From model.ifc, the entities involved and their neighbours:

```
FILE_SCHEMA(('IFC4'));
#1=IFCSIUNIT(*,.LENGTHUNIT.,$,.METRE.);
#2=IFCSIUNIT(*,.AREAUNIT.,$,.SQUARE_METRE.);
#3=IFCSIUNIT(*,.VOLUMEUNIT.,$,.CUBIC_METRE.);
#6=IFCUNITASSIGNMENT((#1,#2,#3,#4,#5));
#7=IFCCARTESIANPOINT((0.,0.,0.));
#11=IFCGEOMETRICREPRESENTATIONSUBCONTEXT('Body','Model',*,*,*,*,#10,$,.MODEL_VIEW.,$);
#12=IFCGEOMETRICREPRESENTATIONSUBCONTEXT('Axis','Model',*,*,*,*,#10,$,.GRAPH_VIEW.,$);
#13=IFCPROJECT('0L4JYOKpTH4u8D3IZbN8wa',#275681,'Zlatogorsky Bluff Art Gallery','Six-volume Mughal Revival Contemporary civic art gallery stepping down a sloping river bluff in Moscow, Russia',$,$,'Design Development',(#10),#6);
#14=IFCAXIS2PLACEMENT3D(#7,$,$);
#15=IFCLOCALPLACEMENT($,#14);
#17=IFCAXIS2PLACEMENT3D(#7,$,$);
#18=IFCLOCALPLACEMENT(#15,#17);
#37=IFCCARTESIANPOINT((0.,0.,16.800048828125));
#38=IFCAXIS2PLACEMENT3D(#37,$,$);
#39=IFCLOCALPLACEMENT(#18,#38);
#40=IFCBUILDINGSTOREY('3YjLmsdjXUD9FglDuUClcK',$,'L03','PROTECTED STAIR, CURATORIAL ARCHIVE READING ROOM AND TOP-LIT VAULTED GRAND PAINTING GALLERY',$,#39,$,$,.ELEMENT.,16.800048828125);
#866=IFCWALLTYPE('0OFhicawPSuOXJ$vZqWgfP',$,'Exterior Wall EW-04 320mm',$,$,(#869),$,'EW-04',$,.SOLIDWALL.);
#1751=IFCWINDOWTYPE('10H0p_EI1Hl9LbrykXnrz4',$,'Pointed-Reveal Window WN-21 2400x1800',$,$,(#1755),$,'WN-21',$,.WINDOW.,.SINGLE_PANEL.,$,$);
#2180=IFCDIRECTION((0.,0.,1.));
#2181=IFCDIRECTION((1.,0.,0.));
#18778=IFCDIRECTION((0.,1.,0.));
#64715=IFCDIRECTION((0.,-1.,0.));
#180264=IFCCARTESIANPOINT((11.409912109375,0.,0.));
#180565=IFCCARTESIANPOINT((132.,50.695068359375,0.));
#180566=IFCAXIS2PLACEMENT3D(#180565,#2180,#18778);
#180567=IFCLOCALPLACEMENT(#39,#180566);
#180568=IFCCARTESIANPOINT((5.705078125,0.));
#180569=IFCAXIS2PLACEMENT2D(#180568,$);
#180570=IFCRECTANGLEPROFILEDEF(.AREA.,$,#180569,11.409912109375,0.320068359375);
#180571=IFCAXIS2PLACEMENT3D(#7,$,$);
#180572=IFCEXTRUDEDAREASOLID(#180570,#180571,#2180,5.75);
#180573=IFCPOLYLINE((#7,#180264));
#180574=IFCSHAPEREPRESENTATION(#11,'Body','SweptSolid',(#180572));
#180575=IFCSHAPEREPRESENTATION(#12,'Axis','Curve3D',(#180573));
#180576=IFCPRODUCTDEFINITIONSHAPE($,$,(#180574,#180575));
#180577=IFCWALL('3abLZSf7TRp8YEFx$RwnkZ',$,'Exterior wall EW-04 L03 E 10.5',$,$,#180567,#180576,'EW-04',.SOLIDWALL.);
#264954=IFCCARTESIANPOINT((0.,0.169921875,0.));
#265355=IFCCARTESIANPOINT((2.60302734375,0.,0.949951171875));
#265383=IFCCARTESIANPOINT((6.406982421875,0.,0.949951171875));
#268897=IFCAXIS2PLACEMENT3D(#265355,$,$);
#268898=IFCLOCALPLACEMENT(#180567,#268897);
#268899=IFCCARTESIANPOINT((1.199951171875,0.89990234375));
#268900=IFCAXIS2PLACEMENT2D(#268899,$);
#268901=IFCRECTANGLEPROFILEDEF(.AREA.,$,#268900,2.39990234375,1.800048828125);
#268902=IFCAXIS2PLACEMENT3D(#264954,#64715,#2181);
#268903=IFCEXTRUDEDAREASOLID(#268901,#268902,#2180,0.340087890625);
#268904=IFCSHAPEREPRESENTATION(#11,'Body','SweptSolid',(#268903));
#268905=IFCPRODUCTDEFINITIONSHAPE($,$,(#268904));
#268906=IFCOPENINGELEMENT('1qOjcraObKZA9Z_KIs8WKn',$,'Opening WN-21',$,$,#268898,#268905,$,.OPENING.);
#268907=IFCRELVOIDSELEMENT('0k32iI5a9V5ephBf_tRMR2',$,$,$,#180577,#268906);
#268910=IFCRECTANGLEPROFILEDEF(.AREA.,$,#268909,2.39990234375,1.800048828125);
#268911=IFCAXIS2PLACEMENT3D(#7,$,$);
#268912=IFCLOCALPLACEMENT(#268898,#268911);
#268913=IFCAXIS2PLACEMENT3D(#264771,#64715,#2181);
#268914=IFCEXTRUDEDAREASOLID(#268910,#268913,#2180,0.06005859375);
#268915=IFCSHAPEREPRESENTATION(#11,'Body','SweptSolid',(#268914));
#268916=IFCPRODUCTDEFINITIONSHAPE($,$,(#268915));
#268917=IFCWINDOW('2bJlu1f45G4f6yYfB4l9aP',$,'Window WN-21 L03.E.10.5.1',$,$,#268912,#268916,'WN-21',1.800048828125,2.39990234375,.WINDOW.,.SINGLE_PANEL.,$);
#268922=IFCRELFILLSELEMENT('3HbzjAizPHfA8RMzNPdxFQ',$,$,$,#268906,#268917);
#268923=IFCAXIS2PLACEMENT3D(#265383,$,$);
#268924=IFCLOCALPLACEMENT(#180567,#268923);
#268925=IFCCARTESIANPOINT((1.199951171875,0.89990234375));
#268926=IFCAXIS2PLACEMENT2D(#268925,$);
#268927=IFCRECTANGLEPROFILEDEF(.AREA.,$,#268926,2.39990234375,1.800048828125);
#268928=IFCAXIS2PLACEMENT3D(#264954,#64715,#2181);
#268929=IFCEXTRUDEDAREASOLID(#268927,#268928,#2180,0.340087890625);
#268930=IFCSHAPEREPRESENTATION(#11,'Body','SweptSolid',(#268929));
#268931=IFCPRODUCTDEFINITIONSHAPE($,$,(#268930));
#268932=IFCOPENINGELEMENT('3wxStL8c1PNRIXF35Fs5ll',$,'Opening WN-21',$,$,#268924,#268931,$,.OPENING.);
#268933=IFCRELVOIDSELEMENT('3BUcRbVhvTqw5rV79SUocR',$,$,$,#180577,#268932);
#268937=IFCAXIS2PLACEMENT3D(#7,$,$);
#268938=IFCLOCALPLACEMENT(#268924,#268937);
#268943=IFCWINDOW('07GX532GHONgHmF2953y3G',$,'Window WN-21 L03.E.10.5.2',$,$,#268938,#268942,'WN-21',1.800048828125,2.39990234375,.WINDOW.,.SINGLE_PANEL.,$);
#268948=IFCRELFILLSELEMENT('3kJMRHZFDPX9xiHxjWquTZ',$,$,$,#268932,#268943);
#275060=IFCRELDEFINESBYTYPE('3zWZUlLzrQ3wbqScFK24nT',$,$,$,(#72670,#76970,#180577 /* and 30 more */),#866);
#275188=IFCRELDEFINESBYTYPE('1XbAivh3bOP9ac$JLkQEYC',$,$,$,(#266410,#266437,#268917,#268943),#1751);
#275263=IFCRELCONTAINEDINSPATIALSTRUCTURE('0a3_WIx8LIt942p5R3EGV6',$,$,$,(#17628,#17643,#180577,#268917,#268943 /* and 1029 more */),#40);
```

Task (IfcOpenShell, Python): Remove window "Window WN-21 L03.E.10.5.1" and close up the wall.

```python
import ifcopenshell
import ifcopenshell.api.feature
import ifcopenshell.api.root
import ifcopenshell.geom
import ifcopenshell.util.shape

model = ifcopenshell.open("model.ifc")
settings = ifcopenshell.geom.settings()


def volume(element):
    """Net volume in cubic metres, openings subtracted."""
    shape = ifcopenshell.geom.create_shape(settings, element)
    return ifcopenshell.util.shape.get_volume(shape.geometry)


window = model.by_guid("2bJlu1f45G4f6yYfB4l9aP")
opening = window.FillsVoids[0].RelatingOpeningElement
wall = opening.VoidsElements[0].RelatingBuildingElement
before = volume(wall)

ifcopenshell.api.root.remove_product(model, product=window)
ifcopenshell.api.feature.remove_feature(model, feature=opening)

after = volume(wall)

print(f"wall volume {before:.3f} -> {after:.3f} m3")

model.write("model_edited.ifc")
```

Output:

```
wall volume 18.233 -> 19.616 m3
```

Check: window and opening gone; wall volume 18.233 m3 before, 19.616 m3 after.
